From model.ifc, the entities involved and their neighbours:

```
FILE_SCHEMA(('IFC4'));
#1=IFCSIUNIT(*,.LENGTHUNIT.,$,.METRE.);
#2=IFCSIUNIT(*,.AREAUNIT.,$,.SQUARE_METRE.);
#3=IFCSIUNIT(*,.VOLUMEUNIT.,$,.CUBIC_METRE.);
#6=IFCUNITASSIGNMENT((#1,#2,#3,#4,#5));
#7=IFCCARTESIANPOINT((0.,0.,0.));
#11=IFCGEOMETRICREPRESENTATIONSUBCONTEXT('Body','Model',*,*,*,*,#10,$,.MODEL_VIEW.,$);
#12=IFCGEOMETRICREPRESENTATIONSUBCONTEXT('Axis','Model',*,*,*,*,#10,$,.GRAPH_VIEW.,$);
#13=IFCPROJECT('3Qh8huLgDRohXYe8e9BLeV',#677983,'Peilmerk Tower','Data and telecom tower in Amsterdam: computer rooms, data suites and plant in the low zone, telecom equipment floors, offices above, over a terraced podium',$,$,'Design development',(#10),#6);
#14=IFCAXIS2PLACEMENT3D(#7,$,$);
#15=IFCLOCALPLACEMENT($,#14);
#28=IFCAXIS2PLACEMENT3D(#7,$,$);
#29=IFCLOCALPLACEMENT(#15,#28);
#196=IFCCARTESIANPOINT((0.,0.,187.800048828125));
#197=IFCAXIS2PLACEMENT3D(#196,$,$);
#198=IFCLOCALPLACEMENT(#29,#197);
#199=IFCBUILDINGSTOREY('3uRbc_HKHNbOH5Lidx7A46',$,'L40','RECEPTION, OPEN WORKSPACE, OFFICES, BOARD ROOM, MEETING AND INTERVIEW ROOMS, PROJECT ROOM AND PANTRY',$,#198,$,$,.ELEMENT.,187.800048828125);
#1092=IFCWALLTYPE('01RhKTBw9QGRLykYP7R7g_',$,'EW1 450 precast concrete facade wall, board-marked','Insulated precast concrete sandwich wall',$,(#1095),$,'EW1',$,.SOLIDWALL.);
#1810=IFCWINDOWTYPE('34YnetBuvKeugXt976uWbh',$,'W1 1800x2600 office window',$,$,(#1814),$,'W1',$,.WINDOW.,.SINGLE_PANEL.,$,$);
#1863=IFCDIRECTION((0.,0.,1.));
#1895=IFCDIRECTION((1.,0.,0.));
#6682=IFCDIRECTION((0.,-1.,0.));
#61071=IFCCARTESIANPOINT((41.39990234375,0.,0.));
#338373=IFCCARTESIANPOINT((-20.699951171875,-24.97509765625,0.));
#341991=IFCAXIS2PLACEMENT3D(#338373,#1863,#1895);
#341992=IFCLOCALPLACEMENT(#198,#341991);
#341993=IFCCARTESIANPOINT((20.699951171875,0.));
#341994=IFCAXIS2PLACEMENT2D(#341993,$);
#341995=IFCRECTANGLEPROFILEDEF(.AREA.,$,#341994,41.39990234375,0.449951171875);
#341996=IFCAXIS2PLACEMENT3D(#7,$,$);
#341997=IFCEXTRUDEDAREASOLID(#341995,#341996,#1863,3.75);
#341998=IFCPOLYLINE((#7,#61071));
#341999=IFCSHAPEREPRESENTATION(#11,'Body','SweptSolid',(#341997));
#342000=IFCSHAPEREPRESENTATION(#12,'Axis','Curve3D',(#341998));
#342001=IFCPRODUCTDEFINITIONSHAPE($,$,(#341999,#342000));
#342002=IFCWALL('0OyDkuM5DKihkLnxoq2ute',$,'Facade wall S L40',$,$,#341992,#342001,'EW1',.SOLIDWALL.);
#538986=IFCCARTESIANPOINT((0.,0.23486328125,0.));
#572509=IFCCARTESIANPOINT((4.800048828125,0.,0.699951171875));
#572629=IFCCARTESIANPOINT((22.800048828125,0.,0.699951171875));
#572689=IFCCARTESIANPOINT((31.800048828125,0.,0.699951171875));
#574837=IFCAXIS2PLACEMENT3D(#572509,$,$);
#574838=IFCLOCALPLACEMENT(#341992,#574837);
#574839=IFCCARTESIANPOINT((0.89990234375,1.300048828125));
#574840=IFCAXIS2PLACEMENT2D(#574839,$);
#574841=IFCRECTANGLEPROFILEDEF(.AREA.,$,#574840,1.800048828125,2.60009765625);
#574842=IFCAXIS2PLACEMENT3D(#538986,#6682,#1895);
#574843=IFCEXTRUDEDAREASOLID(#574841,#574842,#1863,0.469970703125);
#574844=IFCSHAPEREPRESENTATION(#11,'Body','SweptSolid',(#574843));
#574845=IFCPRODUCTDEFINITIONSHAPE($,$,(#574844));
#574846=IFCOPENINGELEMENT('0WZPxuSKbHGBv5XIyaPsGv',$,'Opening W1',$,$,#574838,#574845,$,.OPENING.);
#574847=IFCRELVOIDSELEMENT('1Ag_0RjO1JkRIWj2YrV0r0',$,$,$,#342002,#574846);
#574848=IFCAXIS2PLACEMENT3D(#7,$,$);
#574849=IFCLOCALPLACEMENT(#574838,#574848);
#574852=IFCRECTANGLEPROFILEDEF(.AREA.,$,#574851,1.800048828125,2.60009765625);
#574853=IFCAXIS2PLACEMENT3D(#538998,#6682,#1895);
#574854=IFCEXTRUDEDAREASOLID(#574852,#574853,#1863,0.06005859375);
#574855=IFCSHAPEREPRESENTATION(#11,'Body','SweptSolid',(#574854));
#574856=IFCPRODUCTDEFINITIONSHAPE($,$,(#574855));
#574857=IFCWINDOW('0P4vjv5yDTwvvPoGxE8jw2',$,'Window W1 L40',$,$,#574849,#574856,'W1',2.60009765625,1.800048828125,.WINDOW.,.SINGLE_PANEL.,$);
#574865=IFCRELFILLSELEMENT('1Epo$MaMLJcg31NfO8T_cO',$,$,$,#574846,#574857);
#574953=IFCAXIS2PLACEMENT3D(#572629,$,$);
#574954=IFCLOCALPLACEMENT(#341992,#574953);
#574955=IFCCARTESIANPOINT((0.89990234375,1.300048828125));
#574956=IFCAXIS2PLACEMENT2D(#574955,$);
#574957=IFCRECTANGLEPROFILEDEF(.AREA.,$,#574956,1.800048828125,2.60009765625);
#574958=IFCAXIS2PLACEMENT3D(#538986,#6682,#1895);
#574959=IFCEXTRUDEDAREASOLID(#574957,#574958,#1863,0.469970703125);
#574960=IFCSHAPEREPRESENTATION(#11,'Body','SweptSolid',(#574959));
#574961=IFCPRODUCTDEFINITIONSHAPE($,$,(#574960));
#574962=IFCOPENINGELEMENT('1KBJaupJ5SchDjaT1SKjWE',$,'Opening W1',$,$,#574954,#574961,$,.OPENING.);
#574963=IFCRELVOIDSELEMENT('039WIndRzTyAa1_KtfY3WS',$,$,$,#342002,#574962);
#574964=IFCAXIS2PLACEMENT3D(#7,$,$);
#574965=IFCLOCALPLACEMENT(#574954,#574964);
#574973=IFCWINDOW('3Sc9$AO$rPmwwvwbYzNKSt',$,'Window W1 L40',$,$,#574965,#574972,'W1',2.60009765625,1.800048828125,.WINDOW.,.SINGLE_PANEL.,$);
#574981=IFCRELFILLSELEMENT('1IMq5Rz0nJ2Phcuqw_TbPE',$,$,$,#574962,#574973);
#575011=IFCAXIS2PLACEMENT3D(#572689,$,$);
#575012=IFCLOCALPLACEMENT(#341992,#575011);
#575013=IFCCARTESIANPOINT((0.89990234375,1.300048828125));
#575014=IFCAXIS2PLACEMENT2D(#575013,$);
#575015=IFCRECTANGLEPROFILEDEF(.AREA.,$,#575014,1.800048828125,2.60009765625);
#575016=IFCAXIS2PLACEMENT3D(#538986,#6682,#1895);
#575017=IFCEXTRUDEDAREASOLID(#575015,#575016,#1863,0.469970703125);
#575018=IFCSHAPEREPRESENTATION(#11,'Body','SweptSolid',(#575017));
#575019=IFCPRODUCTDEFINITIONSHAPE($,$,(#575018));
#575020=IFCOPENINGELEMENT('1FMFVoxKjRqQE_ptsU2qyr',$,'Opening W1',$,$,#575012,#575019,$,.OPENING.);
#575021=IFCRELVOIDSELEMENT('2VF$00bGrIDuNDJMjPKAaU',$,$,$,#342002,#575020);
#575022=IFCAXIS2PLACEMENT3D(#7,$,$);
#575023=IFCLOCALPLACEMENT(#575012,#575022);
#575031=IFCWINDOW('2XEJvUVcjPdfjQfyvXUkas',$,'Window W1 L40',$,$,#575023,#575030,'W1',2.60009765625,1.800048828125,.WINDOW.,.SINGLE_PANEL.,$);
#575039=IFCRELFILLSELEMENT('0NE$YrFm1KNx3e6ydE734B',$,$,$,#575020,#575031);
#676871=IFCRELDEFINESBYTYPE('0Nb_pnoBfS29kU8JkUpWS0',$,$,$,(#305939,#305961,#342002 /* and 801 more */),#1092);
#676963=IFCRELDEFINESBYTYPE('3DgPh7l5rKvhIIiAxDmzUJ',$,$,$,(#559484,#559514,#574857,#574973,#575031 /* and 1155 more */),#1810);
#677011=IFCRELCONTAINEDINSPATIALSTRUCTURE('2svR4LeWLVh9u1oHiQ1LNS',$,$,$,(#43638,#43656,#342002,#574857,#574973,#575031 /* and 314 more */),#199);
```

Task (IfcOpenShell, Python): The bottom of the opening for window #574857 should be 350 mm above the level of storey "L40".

```python
import numpy as np
import ifcopenshell
import ifcopenshell.api.geometry
import ifcopenshell.geom
import ifcopenshell.util.element
import ifcopenshell.util.placement
import ifcopenshell.util.shape
import ifcopenshell.util.unit

model = ifcopenshell.open("model.ifc")
unit_scale = ifcopenshell.util.unit.calculate_unit_scale(model)

window = model.by_id(574857)
opening = window.FillsVoids[0].RelatingOpeningElement
storey = ifcopenshell.util.element.get_container(window, ifc_class="IfcBuildingStorey")
level = ifcopenshell.util.placement.get_local_placement(storey.ObjectPlacement)[2, 3]

# The opening's origin need not be at the sill, so measure its lowest point.
shape = ifcopenshell.geom.create_shape(ifcopenshell.geom.settings(), opening)
bottom = ifcopenshell.util.shape.get_shape_bottom_elevation(shape, shape.geometry) / unit_scale
dz = level + 0.35 / unit_scale - bottom

shift = np.array([0.0, 0.0, dz])
# The window is placed relative to its opening, so it follows when the opening moves.
matrix = ifcopenshell.util.placement.get_local_placement(opening.ObjectPlacement)
matrix[:3, 3] += shift
ifcopenshell.api.geometry.edit_object_placement(
    model, product=opening, matrix=matrix, is_si=False, should_transform_children=True
)

print(f"moved by {dz * unit_scale:+.3f} m")

model.write("model-out.ifc")
```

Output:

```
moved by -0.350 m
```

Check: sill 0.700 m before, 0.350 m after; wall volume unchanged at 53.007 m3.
